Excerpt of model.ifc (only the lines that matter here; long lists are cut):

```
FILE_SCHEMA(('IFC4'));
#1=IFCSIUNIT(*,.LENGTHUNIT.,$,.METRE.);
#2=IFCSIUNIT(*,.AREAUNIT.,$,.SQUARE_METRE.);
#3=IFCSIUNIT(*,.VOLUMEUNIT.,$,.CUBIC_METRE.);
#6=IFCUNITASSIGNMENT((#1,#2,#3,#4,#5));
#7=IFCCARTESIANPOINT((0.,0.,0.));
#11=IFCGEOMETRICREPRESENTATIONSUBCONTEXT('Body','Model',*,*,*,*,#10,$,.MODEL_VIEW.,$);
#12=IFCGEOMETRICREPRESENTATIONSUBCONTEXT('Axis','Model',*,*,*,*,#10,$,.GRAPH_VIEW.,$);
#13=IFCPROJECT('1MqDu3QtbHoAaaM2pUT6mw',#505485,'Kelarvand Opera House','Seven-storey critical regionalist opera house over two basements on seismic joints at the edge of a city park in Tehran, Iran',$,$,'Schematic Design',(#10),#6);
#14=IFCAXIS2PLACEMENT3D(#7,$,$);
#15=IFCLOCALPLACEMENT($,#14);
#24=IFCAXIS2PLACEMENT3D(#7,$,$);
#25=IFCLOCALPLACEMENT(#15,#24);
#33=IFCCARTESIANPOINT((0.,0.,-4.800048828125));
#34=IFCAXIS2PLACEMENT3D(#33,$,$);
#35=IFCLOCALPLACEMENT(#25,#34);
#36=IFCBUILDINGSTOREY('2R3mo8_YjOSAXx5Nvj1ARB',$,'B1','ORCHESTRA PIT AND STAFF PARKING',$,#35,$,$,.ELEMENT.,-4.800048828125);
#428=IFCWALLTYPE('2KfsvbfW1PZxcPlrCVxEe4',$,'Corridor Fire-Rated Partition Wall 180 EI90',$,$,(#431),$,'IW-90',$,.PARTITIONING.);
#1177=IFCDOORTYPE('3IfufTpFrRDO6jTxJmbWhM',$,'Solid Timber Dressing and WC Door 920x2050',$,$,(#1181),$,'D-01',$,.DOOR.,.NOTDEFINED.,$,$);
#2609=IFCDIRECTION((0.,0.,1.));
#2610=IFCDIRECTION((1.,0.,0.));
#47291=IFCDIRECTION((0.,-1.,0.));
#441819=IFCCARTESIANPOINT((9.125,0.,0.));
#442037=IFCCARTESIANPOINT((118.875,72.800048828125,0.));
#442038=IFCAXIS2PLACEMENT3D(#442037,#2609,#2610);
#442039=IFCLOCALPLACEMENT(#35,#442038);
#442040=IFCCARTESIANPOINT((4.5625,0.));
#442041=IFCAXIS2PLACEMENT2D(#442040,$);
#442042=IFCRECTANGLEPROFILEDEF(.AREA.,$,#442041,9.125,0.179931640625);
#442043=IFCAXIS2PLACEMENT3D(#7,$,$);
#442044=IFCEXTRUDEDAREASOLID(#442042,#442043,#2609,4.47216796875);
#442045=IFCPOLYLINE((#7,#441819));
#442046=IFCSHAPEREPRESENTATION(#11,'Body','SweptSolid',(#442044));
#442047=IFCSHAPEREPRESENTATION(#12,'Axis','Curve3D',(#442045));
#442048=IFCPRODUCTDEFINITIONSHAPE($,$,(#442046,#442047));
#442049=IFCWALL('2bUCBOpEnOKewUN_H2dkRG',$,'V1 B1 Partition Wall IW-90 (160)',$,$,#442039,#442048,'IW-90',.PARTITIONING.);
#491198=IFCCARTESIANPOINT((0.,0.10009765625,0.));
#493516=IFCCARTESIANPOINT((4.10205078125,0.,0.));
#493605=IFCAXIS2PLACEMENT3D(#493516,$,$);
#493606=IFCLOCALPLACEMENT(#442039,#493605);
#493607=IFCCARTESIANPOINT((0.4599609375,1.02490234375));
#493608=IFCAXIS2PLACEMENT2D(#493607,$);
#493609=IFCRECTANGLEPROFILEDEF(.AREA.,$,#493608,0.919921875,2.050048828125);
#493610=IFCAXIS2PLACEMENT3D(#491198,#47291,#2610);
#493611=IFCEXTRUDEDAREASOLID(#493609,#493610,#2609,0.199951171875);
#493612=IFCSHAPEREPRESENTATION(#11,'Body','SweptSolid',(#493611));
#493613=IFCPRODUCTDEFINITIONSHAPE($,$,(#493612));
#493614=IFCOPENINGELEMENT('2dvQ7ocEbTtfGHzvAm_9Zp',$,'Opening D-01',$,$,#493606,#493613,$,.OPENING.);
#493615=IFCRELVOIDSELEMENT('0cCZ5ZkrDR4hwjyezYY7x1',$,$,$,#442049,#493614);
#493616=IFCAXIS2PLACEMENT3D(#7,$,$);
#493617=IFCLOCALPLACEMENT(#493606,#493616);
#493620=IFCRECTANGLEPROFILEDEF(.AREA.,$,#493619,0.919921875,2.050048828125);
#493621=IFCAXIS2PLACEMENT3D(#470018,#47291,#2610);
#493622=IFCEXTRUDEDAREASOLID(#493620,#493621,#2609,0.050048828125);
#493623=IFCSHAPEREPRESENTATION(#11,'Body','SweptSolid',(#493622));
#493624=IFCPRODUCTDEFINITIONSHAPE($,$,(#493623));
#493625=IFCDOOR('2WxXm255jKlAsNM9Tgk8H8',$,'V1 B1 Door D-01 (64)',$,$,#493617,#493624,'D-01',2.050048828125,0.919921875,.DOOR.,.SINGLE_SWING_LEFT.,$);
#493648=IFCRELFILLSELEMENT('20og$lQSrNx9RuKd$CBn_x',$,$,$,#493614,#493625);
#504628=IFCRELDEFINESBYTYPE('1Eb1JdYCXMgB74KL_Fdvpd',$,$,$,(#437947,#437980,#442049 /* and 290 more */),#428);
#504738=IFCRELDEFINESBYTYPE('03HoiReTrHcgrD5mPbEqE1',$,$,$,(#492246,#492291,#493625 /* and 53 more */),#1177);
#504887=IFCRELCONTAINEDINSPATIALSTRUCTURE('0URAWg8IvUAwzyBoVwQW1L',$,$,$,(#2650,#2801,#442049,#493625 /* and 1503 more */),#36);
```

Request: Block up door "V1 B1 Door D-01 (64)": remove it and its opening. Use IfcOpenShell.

```python
import ifcopenshell
import ifcopenshell.api.feature
import ifcopenshell.api.root
import ifcopenshell.geom
import ifcopenshell.util.shape

model = ifcopenshell.open("model.ifc")
settings = ifcopenshell.geom.settings()


def volume(element):
    """Net volume in cubic metres, openings subtracted."""
    shape = ifcopenshell.geom.create_shape(settings, element)
    return ifcopenshell.util.shape.get_volume(shape.geometry)


door = model.by_guid("2WxXm255jKlAsNM9Tgk8H8")
opening = door.FillsVoids[0].RelatingOpeningElement
wall = opening.VoidsElements[0].RelatingBuildingElement
before = volume(wall)

ifcopenshell.api.root.remove_product(model, product=door)
ifcopenshell.api.feature.remove_feature(model, feature=opening)

after = volume(wall)

print(f"wall volume {before:.3f} -> {after:.3f} m3")

model.write("model_rev.ifc")
```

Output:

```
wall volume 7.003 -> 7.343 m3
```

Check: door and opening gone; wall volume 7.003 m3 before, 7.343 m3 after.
